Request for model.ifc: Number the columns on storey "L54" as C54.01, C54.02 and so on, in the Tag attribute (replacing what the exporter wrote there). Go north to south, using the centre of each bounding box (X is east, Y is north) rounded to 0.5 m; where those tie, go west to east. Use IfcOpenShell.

First a look at what the model holds.

```python
import ifcopenshell
import ifcopenshell.util.element
import ifcopenshell.util.placement

model = ifcopenshell.open("model.ifc")
print(model.schema)
storey = next(s for s in model.by_type("IfcBuildingStorey") if s.Name == "L54")
columns = [e for e in ifcopenshell.util.element.get_decomposition(storey) if e.is_a("IfcColumn")]
for e in sorted(columns, key=lambda e: e.id()):
    origin = ifcopenshell.util.placement.get_local_placement(e.ObjectPlacement)[:3, 3]
    print(e.id(), e.Tag, e.Name, origin.round(2) + 0.0, sep=" | ")
```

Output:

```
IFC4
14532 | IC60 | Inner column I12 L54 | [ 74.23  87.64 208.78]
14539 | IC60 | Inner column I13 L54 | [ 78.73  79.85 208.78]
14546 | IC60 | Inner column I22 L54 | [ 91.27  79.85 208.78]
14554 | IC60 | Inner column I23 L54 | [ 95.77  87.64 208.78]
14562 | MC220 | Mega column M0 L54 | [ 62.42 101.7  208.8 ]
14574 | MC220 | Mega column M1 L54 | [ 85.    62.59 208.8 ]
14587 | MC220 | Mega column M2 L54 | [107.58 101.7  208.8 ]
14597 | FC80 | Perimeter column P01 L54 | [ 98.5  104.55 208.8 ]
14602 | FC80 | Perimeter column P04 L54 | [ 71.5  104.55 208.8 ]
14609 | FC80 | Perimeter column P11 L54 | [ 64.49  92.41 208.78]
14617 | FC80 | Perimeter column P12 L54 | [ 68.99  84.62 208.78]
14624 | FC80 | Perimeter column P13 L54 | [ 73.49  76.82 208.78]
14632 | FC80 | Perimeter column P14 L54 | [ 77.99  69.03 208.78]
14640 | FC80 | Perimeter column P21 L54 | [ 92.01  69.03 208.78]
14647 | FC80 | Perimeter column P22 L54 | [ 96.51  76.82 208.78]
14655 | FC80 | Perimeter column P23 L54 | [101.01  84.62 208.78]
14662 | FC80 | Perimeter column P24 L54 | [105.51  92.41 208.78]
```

```python
import ifcopenshell
import ifcopenshell.geom
import ifcopenshell.util.element
import ifcopenshell.util.shape

model = ifcopenshell.open("model.ifc")
settings = ifcopenshell.geom.settings()
settings.set("use-world-coords", True)


def centre(element):
    shape = ifcopenshell.geom.create_shape(settings, element)
    return ifcopenshell.util.shape.get_bbox_centroid(shape.geometry)


storey = next(s for s in model.by_type("IfcBuildingStorey") if s.Name == "L54")
columns = [e for e in ifcopenshell.util.element.get_decomposition(storey) if e.is_a("IfcColumn")]

# Insertion points can sit at a corner or the storey origin, so sort by the geometry (in metres).
centres = {e: centre(e) for e in columns}
columns.sort(key=lambda e: (-round(centres[e][1] / 0.5), centres[e][0]))

for i, e in enumerate(columns, start=1):
    number = f"C54.{i:02d}"
    e.Tag = number
    print(e.id(), number)

model.write("model-out.ifc")
```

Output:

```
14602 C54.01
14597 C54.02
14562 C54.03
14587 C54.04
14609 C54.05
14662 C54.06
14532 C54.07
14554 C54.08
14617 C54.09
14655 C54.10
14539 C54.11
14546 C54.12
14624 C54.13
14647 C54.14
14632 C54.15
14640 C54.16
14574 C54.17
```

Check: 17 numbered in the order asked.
